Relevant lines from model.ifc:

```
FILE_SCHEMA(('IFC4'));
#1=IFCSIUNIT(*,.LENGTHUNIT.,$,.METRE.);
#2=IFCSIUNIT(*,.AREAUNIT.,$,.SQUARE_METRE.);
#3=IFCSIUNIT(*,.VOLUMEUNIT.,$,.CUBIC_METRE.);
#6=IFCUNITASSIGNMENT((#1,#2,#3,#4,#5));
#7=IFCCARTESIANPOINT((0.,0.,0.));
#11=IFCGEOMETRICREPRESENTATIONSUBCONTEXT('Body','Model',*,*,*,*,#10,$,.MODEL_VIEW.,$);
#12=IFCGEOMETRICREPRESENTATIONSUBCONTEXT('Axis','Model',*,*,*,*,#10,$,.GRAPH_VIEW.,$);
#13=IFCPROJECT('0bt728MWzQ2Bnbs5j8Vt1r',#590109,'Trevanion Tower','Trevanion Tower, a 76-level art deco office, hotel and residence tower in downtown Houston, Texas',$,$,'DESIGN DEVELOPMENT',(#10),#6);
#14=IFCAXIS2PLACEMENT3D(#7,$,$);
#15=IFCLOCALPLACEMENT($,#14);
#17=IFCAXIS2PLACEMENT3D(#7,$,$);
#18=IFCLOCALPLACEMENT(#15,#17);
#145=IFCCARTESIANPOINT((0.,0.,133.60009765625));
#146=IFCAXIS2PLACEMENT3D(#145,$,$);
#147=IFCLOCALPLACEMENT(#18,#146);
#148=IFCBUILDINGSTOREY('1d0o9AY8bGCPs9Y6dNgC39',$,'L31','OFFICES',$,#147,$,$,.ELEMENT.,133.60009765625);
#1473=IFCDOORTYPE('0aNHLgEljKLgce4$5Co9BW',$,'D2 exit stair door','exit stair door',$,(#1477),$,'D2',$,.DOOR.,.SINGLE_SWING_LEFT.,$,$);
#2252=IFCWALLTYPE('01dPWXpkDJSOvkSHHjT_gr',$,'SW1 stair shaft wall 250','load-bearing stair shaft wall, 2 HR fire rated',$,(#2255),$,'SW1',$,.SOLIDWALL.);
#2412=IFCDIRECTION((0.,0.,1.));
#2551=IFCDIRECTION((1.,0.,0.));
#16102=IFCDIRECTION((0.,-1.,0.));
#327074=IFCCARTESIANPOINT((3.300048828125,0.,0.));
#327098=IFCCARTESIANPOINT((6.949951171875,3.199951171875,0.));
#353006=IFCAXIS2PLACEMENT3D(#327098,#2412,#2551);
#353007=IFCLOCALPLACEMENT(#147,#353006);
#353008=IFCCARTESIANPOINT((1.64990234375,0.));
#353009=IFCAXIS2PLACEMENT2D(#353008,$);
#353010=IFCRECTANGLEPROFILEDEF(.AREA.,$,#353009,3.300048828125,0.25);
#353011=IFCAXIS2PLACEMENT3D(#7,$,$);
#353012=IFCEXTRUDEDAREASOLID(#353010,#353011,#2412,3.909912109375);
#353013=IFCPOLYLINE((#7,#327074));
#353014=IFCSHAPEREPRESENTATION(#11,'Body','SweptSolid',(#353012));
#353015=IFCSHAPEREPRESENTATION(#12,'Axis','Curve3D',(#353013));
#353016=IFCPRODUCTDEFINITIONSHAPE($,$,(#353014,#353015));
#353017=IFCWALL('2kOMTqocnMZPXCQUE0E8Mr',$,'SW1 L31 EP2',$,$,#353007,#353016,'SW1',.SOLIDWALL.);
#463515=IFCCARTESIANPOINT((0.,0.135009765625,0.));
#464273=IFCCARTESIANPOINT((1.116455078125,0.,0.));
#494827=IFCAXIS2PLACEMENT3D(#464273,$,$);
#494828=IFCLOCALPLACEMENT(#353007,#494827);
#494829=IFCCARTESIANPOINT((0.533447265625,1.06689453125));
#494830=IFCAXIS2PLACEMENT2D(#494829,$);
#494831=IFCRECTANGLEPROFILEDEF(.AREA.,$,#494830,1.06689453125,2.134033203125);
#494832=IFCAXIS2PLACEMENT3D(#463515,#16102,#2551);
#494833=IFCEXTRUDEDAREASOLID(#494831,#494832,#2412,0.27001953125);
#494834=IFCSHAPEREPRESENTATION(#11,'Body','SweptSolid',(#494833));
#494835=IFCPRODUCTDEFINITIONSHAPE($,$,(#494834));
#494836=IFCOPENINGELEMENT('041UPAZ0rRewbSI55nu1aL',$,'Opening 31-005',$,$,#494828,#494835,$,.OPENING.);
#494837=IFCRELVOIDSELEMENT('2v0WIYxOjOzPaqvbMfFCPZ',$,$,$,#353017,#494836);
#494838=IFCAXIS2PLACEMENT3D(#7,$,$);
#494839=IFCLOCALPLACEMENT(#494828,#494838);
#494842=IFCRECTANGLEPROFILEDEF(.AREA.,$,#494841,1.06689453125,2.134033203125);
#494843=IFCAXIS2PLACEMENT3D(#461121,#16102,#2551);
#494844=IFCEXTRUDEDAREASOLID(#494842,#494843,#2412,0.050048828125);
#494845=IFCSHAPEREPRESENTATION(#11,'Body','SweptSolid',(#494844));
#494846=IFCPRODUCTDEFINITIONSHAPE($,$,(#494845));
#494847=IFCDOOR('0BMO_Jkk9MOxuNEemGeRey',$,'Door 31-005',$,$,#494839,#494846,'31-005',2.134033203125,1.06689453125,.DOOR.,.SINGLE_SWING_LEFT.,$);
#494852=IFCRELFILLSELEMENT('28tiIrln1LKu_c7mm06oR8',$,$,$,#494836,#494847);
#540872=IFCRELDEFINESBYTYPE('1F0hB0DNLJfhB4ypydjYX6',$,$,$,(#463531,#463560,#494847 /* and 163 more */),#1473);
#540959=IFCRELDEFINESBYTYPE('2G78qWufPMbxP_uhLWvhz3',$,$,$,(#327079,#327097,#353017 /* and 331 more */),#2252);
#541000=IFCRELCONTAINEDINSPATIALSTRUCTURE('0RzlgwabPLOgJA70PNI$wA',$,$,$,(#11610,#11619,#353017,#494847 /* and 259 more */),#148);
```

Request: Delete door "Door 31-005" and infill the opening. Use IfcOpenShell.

```python
import ifcopenshell
import ifcopenshell.api.feature
import ifcopenshell.api.root
import ifcopenshell.geom
import ifcopenshell.util.shape

model = ifcopenshell.open("model.ifc")
settings = ifcopenshell.geom.settings()


def volume(element):
    """Net volume in cubic metres, openings subtracted."""
    shape = ifcopenshell.geom.create_shape(settings, element)
    return ifcopenshell.util.shape.get_volume(shape.geometry)


door = model.by_id(494847)
opening = door.FillsVoids[0].RelatingOpeningElement
wall = opening.VoidsElements[0].RelatingBuildingElement
before = volume(wall)

ifcopenshell.api.root.remove_product(model, product=door)
ifcopenshell.api.feature.remove_feature(model, feature=opening)

after = volume(wall)

print(f"wall volume {before:.3f} -> {after:.3f} m3")

model.write("model_rev.ifc")
```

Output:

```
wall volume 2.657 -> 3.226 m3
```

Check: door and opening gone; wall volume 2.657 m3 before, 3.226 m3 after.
